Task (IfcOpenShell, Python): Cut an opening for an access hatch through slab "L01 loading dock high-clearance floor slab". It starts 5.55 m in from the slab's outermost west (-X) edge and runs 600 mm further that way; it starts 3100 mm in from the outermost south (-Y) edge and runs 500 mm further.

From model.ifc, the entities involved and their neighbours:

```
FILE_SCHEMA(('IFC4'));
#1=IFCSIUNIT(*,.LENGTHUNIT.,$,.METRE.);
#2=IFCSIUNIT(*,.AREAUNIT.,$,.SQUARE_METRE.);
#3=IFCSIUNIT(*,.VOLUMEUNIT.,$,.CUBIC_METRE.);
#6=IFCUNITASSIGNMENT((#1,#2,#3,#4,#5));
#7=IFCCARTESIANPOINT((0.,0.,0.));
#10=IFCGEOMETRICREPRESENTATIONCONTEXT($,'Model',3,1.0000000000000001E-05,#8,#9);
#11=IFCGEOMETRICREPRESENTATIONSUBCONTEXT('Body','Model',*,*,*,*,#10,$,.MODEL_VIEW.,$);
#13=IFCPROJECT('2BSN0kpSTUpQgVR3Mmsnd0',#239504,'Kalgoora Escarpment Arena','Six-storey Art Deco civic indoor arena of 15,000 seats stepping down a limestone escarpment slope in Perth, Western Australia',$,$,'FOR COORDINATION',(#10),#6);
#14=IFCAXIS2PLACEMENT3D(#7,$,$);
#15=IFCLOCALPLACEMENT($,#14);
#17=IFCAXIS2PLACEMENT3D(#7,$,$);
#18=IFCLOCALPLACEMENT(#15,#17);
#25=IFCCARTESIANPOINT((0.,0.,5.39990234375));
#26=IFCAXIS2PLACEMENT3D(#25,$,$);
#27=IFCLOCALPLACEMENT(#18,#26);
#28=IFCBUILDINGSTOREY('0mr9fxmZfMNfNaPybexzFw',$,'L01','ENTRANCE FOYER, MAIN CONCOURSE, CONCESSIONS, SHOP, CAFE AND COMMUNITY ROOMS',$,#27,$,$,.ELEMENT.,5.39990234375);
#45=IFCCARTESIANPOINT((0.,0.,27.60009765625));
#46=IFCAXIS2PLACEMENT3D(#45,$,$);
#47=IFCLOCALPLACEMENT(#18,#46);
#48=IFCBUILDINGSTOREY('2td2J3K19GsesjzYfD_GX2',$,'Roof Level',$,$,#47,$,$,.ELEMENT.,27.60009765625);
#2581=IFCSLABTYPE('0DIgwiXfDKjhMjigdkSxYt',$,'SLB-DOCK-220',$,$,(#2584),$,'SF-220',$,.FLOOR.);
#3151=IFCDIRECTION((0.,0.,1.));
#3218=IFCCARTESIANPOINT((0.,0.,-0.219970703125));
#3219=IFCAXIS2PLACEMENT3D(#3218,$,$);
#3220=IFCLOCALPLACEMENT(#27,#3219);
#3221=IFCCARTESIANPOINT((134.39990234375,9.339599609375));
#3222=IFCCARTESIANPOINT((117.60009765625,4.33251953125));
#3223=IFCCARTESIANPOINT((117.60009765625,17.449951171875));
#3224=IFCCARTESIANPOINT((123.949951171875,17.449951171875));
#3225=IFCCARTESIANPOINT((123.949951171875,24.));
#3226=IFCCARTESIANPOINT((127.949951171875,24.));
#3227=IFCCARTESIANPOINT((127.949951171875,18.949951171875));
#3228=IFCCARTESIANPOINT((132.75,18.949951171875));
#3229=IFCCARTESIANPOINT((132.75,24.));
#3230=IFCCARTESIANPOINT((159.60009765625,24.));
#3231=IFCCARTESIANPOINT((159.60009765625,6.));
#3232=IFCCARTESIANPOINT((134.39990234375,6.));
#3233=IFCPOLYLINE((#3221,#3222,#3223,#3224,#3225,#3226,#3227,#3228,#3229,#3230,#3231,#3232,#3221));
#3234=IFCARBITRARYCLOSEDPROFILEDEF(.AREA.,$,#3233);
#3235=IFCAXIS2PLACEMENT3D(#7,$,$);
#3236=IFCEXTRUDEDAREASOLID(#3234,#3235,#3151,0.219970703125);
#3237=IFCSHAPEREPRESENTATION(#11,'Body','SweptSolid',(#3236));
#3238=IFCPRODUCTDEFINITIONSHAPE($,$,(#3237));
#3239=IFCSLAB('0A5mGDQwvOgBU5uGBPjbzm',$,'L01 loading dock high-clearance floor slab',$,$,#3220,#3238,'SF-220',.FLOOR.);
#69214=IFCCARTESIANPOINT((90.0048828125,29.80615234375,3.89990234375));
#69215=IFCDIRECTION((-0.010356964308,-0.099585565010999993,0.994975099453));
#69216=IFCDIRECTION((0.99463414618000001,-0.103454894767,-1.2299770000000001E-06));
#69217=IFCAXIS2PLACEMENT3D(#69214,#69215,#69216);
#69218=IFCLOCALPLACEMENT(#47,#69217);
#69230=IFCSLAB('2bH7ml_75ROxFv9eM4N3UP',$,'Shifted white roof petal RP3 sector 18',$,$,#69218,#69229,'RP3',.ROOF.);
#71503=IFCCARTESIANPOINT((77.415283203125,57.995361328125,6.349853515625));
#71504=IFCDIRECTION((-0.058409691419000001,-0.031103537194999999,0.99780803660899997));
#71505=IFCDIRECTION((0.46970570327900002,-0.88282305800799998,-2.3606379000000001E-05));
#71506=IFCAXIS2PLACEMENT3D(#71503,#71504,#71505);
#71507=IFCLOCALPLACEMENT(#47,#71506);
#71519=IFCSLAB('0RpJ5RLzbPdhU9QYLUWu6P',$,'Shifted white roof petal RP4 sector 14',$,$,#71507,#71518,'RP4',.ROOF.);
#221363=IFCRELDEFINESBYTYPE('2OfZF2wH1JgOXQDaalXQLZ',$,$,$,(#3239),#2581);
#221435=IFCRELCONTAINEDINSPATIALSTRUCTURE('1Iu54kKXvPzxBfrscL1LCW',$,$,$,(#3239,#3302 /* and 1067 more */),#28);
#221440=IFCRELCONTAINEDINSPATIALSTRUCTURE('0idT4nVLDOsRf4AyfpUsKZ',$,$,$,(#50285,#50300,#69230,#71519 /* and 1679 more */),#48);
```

```python
import numpy as np
import ifcopenshell
import ifcopenshell.api.feature
import ifcopenshell.api.geometry
import ifcopenshell.api.root
import ifcopenshell.geom
import ifcopenshell.util.placement
import ifcopenshell.util.representation
import ifcopenshell.util.shape
import ifcopenshell.util.unit

model = ifcopenshell.open("model.ifc")
unit_scale = ifcopenshell.util.unit.calculate_unit_scale(model)
settings = ifcopenshell.geom.settings()


def volume(element):
    """Net volume in cubic metres, openings subtracted."""
    shape = ifcopenshell.geom.create_shape(settings, element)
    return ifcopenshell.util.shape.get_volume(shape.geometry)


slab = model.by_id(3239)
before = volume(slab)

# Extent in the slab's own axes, in metres. The edges named are its -X and -Y sides.
slab_shape = ifcopenshell.geom.create_shape(settings, slab)
vertices = ifcopenshell.util.shape.get_vertices(slab_shape.geometry)
x_min, y_min, bottom = vertices.min(axis=0)
top = vertices[:, 2].max()

opening = ifcopenshell.api.root.create_entity(model, ifc_class="IfcOpeningElement", name="Access hatch opening", predefined_type="OPENING")
context = ifcopenshell.util.representation.get_context(model, "Model", "Body", "MODEL_VIEW")
width, depth = 0.6, 0.5
outline = [(0.0, 0.0), (width, 0.0), (width, depth), (0.0, depth), (0.0, 0.0)]
# Overshoot both faces by 50 mm so the cut is clean.
shape = ifcopenshell.api.geometry.add_slab_representation(
    model, context=context, depth=top - bottom + 0.1, polyline=outline
)
ifcopenshell.api.geometry.assign_representation(model, product=opening, representation=shape)

matrix = ifcopenshell.util.placement.get_local_placement(slab.ObjectPlacement)
matrix[:, 3] = matrix @ np.append(np.array([x_min + 5.55, y_min + 3.1, bottom - 0.05]) / unit_scale, 1.0)
ifcopenshell.api.geometry.edit_object_placement(model, product=opening, matrix=matrix, is_si=False)
ifcopenshell.api.feature.add_feature(model, feature=opening, element=slab)

after = volume(slab)

print(f"slab volume {before:.3f} -> {after:.3f} m3")

model.write("model_updated.ifc")
```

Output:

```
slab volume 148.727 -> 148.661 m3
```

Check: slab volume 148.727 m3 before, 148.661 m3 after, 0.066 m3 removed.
